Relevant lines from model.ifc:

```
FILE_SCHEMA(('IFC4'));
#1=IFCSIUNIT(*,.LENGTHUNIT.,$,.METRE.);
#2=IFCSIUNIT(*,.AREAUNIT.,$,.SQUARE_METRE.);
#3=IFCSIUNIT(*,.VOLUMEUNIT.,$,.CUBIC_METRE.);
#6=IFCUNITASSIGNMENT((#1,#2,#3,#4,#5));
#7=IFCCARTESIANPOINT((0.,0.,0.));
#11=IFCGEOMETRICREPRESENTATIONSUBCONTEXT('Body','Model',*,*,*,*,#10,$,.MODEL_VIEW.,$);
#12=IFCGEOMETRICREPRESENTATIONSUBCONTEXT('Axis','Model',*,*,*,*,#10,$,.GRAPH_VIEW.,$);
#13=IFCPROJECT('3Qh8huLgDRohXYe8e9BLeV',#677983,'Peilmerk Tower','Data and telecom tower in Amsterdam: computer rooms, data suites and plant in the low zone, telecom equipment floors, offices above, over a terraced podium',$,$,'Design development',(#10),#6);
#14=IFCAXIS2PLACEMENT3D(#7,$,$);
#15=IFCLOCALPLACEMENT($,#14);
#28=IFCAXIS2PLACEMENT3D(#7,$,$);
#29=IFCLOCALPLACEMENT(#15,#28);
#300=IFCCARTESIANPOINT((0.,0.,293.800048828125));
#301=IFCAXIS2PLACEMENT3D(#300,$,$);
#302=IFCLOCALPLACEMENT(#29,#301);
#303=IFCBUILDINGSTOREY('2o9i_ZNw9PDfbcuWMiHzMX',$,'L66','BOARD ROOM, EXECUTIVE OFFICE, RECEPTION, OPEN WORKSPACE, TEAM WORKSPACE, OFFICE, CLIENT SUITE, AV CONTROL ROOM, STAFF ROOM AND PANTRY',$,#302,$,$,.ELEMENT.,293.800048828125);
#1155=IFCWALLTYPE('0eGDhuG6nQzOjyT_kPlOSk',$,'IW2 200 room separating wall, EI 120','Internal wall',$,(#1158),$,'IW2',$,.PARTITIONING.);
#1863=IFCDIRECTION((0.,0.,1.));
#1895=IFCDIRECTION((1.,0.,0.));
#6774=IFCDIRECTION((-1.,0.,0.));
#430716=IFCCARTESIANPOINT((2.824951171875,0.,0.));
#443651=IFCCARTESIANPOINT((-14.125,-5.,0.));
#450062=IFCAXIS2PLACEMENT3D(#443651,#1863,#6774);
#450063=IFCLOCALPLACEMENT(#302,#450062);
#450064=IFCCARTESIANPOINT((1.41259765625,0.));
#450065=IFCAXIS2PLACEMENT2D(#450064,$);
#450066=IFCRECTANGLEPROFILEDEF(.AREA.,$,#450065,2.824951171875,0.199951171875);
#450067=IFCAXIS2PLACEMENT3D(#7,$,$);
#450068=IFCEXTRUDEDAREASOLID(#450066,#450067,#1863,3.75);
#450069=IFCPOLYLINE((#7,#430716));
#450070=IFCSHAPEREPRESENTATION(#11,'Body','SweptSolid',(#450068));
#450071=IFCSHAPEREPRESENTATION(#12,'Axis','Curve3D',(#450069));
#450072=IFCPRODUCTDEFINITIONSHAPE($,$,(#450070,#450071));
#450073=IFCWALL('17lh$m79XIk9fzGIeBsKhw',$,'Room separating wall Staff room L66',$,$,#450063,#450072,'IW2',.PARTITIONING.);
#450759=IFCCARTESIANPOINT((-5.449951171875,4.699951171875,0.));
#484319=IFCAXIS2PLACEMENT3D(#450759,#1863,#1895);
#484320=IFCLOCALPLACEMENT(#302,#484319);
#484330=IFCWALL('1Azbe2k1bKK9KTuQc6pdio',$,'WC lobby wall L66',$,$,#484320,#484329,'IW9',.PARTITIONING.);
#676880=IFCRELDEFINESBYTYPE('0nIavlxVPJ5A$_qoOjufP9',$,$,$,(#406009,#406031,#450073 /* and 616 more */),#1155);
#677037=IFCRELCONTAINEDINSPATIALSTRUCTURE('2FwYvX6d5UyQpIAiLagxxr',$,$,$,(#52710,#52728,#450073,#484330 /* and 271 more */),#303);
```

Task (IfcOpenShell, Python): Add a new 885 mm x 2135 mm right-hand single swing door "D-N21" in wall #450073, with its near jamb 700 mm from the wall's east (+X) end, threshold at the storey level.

```python
import numpy as np
import ifcopenshell
import ifcopenshell.api.feature
import ifcopenshell.api.geometry
import ifcopenshell.api.root
import ifcopenshell.api.spatial
import ifcopenshell.geom
import ifcopenshell.util.element
import ifcopenshell.util.placement
import ifcopenshell.util.representation
import ifcopenshell.util.shape
import ifcopenshell.util.unit

model = ifcopenshell.open("model.ifc")
unit_scale = ifcopenshell.util.unit.calculate_unit_scale(model)
settings = ifcopenshell.geom.settings()


def volume(element):
    """Net volume in cubic metres, openings subtracted."""
    shape = ifcopenshell.geom.create_shape(settings, element)
    return ifcopenshell.util.shape.get_volume(shape.geometry)


wall = model.by_id(450073)
storey = ifcopenshell.util.element.get_container(wall, ifc_class="IfcBuildingStorey")
context = ifcopenshell.util.representation.get_context(model, "Model", "Body", "MODEL_VIEW")
before = volume(wall)

width, height, from_end, sill = 0.885, 2.135, 0.7, 0.0  # metres

# The wall runs along its own X axis, and the end named is its -X end.
wall_shape = ifcopenshell.geom.create_shape(settings, wall)
x, y, z = ifcopenshell.util.shape.get_vertices(wall_shape.geometry).T
start = x.min() + from_end
face, thickness = float(y.min()), float(y.max() - y.min())
wall_matrix = ifcopenshell.util.placement.get_local_placement(wall.ObjectPlacement)
level = ifcopenshell.util.placement.get_local_placement(storey.ObjectPlacement)[2, 3]


def in_wall(x, y):
    """Placement at x, y metres in the wall's axes, at sill height."""
    matrix = wall_matrix.copy()
    matrix[:, 3] = wall_matrix @ np.array([x / unit_scale, y / unit_scale, 0.0, 1.0])
    matrix[2, 3] = level + sill / unit_scale
    return matrix


# Opening: a box that overshoots both wall faces by 50 mm.
opening = ifcopenshell.api.root.create_entity(model, ifc_class="IfcOpeningElement", predefined_type="OPENING")
box = ifcopenshell.api.geometry.add_wall_representation(
    model, context=context, length=width, height=height, thickness=thickness + 0.1
)
ifcopenshell.api.geometry.assign_representation(model, product=opening, representation=box)
ifcopenshell.api.geometry.edit_object_placement(model, product=opening, matrix=in_wall(start, face - 0.05), is_si=False)
ifcopenshell.api.feature.add_feature(model, feature=opening, element=wall)

door = ifcopenshell.api.root.create_entity(model, ifc_class="IfcDoor", name="D-N21", predefined_type="DOOR")
door.OverallWidth, door.OverallHeight = width / unit_scale, height / unit_scale
door.OperationType = "SINGLE_SWING_RIGHT"
body = ifcopenshell.api.geometry.add_door_representation(
    model,
    context=context,
    overall_width=door.OverallWidth,
    overall_height=door.OverallHeight,
    operation_type="SINGLE_SWING_RIGHT",
    lining_properties={"LiningDepth": thickness / unit_scale, "ThresholdDepth": thickness / unit_scale},
)
ifcopenshell.api.geometry.assign_representation(model, product=door, representation=body)
ifcopenshell.api.spatial.assign_container(model, products=[door], relating_structure=storey)
ifcopenshell.api.feature.add_filling(model, opening=opening, element=door)

# The lining spans the wall, so the door starts at the wall face.
ifcopenshell.api.geometry.edit_object_placement(model, product=door, matrix=in_wall(start, face), is_si=False)

after = volume(wall)

print(f"wall volume {before:.3f} -> {after:.3f} m3")

model.write("model_updated.ifc")
```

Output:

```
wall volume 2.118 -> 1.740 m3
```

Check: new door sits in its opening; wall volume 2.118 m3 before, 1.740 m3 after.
